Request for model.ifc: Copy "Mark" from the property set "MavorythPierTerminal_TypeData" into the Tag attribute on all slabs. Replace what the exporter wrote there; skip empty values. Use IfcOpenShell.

First a look at what the model holds.

```python
import ifcopenshell
import ifcopenshell.util.element

model = ifcopenshell.open("model.ifc")
print(model.schema)
slabs = model.by_type("IfcSlab")
print(len(slabs), "slabs")
for e in slabs[:8]:
    source = ifcopenshell.util.element.get_pset(e, "MavorythPierTerminal_TypeData", "Mark")
    target = e.Tag
    print(e.id(), repr(source), repr(target), sep=" | ")
```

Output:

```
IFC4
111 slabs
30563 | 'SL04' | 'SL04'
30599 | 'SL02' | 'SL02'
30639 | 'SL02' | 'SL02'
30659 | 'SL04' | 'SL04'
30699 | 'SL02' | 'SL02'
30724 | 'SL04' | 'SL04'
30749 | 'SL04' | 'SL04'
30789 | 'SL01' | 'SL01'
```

```python
import ifcopenshell
import ifcopenshell.util.element

model = ifcopenshell.open("model.ifc")

count = 0
for e in model.by_type("IfcSlab"):
    value = ifcopenshell.util.element.get_pset(e, "MavorythPierTerminal_TypeData", "Mark")
    current = e.Tag
    if not value or not value.strip() or current == value:
        continue
    e.Tag = value
    count += 1

print(count, "slabs updated")

model.write("model-out.ifc")
```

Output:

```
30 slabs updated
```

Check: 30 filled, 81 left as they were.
